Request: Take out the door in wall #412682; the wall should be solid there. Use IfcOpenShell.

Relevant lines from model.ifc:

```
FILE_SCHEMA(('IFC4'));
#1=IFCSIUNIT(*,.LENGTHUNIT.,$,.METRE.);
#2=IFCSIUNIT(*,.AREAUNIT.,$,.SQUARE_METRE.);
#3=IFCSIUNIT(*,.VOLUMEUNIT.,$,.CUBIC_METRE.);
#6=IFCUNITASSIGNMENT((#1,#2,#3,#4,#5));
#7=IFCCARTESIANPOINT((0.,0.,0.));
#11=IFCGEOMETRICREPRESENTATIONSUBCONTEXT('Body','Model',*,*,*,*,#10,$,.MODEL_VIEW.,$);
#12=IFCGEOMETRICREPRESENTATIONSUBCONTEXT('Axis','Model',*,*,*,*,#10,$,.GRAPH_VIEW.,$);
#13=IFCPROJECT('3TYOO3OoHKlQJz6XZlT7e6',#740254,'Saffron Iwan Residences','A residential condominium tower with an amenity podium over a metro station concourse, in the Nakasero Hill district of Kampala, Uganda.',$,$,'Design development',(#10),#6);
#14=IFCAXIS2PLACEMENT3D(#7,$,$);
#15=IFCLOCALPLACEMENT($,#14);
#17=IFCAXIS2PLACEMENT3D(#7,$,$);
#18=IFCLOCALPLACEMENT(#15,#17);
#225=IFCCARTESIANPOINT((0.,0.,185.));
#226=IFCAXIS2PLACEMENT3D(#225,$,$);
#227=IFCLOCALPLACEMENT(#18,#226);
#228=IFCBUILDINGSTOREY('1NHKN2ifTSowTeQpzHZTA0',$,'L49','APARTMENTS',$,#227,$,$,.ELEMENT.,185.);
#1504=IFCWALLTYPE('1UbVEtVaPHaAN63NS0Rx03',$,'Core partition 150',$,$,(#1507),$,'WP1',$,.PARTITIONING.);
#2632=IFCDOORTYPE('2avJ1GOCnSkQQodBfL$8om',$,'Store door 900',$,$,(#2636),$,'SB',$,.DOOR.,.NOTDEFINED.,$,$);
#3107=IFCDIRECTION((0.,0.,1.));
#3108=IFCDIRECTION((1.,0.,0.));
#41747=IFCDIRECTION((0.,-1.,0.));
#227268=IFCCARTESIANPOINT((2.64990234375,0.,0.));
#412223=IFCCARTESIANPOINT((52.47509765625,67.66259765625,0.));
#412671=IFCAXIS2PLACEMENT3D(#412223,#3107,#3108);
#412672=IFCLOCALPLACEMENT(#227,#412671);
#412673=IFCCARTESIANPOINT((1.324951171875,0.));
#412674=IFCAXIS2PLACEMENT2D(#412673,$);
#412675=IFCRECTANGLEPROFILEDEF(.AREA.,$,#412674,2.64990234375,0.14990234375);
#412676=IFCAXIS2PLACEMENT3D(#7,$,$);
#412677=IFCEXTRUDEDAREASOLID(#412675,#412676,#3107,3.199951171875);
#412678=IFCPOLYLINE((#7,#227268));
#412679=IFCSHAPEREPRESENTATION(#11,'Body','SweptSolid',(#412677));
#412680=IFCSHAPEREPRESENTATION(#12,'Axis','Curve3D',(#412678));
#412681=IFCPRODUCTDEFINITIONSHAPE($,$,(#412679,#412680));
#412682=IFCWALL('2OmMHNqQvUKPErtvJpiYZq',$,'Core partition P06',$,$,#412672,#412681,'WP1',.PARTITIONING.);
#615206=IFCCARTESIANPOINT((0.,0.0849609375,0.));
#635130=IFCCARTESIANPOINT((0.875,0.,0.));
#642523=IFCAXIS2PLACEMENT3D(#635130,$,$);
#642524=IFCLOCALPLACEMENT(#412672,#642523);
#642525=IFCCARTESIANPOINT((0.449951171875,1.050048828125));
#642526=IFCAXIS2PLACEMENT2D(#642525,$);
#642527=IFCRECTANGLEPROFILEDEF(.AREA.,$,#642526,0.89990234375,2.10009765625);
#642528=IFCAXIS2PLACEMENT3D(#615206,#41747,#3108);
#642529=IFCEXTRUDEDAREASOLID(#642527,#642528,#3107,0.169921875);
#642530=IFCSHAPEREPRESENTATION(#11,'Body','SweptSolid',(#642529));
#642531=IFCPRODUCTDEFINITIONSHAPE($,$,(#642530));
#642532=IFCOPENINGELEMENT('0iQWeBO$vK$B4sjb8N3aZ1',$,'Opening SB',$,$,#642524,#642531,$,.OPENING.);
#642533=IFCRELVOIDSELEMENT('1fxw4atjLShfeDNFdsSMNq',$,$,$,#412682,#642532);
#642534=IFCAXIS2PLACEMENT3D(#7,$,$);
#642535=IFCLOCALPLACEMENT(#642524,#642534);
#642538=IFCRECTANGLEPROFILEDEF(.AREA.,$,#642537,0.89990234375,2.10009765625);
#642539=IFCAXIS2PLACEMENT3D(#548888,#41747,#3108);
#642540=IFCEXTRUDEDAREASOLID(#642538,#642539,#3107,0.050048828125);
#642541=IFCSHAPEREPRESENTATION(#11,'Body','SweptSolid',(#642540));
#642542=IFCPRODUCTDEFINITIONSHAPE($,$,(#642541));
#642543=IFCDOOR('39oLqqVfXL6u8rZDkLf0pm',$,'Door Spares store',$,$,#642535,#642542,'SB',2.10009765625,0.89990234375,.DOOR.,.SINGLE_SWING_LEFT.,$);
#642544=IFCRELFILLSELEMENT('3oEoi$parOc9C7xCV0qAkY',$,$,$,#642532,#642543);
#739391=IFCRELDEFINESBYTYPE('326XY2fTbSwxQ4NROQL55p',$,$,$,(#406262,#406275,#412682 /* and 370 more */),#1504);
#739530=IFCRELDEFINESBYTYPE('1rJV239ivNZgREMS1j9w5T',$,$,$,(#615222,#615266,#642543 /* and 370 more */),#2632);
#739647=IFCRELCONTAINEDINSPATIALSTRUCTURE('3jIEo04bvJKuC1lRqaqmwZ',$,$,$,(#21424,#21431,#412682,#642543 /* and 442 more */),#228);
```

```python
import ifcopenshell
import ifcopenshell.api.feature
import ifcopenshell.api.root
import ifcopenshell.geom
import ifcopenshell.util.shape

model = ifcopenshell.open("model.ifc")
settings = ifcopenshell.geom.settings()


def volume(element):
    """Net volume in cubic metres, openings subtracted."""
    shape = ifcopenshell.geom.create_shape(settings, element)
    return ifcopenshell.util.shape.get_volume(shape.geometry)


door = model.by_guid("39oLqqVfXL6u8rZDkLf0pm")
opening = door.FillsVoids[0].RelatingOpeningElement
wall = opening.VoidsElements[0].RelatingBuildingElement
before = volume(wall)

ifcopenshell.api.root.remove_product(model, product=door)
ifcopenshell.api.feature.remove_feature(model, feature=opening)

after = volume(wall)

print(f"wall volume {before:.3f} -> {after:.3f} m3")

model.write("model-out.ifc")
```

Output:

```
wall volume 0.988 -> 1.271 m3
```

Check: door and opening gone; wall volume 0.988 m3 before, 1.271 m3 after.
